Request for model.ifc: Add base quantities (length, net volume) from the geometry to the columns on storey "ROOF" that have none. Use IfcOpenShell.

First a look at what the model holds.

```python
import ifcopenshell
import ifcopenshell.util.element
import ifcopenshell.util.unit

model = ifcopenshell.open("model.ifc")
print(model.schema)
for unit_type in ("LENGTHUNIT", "AREAUNIT", "VOLUMEUNIT"):
    print(unit_type, ifcopenshell.util.unit.calculate_unit_scale(model, unit_type))
storey = next(s for s in model.by_type("IfcBuildingStorey") if s.Name == "ROOF")
columns = [e for e in ifcopenshell.util.element.get_decomposition(storey) if e.is_a("IfcColumn")]
for e in sorted(columns, key=lambda e: e.id()):
    print(e.id(), e.is_a(), e.Name, list(ifcopenshell.util.element.get_psets(e, qtos_only=True)), sep=" | ")
```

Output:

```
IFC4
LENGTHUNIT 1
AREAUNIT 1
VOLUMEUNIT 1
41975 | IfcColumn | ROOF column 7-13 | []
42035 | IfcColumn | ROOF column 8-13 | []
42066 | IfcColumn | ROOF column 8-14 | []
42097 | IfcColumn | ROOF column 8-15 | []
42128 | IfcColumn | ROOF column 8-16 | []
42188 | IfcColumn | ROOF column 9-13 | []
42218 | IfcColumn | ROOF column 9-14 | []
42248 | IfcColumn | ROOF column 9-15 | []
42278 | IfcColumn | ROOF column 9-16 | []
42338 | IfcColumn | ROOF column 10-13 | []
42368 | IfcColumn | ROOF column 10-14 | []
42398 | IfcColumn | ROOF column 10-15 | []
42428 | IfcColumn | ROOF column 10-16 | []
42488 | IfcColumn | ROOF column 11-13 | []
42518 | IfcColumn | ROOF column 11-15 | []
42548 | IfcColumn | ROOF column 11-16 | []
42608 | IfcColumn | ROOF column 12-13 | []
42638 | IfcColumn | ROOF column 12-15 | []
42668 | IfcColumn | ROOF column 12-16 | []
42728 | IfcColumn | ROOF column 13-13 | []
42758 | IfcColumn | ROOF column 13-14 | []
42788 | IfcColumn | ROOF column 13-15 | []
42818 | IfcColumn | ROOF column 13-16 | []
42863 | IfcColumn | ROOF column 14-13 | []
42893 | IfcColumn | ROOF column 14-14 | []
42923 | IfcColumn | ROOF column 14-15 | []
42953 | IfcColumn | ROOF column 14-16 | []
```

```python
import ifcopenshell
import ifcopenshell.api.pset
import ifcopenshell.geom
import ifcopenshell.util.element
import ifcopenshell.util.shape
import ifcopenshell.util.unit

model = ifcopenshell.open("model.ifc")
unit_scale = ifcopenshell.util.unit.calculate_unit_scale(model)
volume_scale = ifcopenshell.util.unit.calculate_unit_scale(model, "VOLUMEUNIT")
settings = ifcopenshell.geom.settings()

storey = next(s for s in model.by_type("IfcBuildingStorey") if s.Name == "ROOF")
columns = [e for e in ifcopenshell.util.element.get_decomposition(storey) if e.is_a("IfcColumn")]

for e in sorted(columns, key=lambda e: e.id()):
    if ifcopenshell.util.element.get_psets(e, qtos_only=True, should_inherit=False):
        continue
    # Geometry comes back in metres, in the element's own axes.
    shape = ifcopenshell.geom.create_shape(settings, e)
    values = {
        "Length": ifcopenshell.util.shape.get_z(shape.geometry) / unit_scale,
        "NetVolume": ifcopenshell.util.shape.get_volume(shape.geometry) / volume_scale,
    }
    qto = ifcopenshell.api.pset.add_qto(model, product=e, name="Qto_ColumnBaseQuantities")
    ifcopenshell.api.pset.edit_qto(model, qto=qto, properties=values)
    print(e.id(), {k: round(v, 3) for k, v in values.items()})

model.write("model_updated.ifc")
```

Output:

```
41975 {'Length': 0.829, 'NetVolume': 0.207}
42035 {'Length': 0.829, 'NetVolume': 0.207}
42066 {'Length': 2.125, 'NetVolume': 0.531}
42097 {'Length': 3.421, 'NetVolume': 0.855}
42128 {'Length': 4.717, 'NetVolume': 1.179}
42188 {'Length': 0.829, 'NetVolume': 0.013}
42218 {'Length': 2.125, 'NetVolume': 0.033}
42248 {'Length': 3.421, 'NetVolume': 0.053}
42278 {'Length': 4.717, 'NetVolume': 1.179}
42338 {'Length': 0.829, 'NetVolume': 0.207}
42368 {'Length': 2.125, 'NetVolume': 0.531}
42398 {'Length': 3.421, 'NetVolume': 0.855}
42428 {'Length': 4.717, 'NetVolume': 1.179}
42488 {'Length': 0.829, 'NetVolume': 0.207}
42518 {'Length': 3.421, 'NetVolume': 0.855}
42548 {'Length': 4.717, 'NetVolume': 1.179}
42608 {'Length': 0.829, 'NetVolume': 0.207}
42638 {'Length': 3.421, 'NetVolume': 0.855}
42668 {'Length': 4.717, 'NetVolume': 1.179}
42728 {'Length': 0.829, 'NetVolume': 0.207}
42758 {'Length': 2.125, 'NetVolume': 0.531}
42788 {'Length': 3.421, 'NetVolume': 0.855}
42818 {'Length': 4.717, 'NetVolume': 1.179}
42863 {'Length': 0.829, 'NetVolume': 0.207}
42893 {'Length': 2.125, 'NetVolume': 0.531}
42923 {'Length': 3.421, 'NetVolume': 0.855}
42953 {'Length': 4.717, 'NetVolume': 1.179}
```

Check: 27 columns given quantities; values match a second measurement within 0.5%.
